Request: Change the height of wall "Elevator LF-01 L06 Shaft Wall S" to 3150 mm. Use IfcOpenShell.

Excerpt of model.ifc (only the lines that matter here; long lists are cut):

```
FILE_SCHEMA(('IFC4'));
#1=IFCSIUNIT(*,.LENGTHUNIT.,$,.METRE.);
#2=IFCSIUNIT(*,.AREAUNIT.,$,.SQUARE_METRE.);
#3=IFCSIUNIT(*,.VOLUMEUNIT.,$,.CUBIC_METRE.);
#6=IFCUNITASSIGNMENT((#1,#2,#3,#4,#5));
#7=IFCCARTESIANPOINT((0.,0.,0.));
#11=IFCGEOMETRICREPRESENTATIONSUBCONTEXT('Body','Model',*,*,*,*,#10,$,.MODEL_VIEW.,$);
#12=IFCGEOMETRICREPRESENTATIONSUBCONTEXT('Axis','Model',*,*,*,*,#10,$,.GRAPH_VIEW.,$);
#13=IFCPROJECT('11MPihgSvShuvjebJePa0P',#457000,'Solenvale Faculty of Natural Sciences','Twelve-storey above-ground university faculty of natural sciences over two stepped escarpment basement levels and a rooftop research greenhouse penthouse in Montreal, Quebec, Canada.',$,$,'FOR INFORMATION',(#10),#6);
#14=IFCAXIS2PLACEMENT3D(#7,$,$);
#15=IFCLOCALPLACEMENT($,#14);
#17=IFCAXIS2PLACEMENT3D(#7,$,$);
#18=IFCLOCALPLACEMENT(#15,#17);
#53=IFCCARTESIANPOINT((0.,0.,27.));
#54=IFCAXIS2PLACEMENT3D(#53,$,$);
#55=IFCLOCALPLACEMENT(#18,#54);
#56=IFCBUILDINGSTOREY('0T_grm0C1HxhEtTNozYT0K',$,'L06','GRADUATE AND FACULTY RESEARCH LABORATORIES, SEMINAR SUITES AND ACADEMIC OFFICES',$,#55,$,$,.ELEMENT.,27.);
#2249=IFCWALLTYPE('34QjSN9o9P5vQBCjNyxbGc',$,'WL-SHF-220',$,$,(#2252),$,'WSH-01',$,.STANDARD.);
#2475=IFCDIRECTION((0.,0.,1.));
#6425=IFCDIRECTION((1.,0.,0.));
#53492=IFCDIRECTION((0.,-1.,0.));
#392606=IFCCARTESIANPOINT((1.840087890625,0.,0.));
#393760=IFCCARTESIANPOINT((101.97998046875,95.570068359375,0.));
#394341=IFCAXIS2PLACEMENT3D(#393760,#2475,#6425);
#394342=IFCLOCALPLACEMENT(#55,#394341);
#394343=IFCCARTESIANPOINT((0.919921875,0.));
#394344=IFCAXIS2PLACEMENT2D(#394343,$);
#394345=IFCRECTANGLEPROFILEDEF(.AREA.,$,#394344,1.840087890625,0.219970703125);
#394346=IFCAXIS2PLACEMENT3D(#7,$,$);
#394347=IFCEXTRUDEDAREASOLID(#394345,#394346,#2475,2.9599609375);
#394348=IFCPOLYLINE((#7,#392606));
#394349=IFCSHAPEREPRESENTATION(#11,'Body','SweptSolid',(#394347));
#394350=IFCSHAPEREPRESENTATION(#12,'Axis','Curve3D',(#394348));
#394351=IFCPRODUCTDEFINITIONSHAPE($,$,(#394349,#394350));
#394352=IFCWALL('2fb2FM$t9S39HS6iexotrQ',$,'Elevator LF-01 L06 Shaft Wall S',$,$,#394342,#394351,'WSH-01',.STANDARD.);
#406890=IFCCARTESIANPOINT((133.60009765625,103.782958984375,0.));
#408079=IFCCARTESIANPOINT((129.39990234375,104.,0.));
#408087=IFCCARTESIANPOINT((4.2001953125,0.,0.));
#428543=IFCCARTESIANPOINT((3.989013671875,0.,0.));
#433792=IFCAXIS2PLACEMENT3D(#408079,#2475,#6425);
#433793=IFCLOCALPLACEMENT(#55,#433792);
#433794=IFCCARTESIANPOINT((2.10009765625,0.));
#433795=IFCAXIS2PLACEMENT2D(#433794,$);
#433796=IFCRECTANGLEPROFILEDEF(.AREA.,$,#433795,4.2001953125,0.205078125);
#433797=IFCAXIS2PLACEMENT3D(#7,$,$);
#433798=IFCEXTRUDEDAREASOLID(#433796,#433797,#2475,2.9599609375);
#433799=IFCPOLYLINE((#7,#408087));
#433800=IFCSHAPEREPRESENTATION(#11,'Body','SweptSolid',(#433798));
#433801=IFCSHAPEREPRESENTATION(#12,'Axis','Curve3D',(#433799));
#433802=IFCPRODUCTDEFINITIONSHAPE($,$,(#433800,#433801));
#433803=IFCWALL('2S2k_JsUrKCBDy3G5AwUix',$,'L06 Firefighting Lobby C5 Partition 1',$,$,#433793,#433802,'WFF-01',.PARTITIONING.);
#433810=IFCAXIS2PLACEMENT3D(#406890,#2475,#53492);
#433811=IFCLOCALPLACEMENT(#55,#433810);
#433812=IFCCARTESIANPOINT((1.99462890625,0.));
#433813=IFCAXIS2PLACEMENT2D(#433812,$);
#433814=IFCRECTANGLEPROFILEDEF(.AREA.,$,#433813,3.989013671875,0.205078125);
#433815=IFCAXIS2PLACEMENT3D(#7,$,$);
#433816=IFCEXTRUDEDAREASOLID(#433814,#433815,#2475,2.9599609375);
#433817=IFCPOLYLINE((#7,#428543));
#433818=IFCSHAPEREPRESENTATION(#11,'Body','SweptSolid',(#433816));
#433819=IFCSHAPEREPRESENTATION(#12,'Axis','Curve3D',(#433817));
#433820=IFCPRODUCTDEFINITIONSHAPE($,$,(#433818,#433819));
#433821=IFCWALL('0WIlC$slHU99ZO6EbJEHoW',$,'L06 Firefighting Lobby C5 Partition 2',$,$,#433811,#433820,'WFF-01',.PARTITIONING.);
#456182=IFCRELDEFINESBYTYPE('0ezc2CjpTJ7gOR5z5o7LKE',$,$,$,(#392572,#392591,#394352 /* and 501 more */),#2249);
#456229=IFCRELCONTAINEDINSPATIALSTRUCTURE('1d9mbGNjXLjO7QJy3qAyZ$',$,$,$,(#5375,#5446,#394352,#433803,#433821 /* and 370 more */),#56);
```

```python
import ifcopenshell
import ifcopenshell.geom
import ifcopenshell.util.representation
import ifcopenshell.util.shape
import ifcopenshell.util.unit

model = ifcopenshell.open("model.ifc")
unit_scale = ifcopenshell.util.unit.calculate_unit_scale(model)
settings = ifcopenshell.geom.settings()


def volume(element):
    """Net volume in cubic metres, openings subtracted."""
    shape = ifcopenshell.geom.create_shape(settings, element)
    return ifcopenshell.util.shape.get_volume(shape.geometry)


wall = model.by_guid("2fb2FM$t9S39HS6iexotrQ")
before = volume(wall)

body = ifcopenshell.util.representation.get_representation(wall, "Model", "Body")
solid = body.Items[0]
old_height = solid.Depth
solid.Depth = 3.15 / unit_scale
after = volume(wall)

print(f"height {old_height:g} -> {solid.Depth:g}, volume {before:.3f} -> {after:.3f} m3")

model.write("model-out.ifc")
```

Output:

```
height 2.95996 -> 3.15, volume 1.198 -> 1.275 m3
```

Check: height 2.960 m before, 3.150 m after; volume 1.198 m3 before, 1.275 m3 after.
